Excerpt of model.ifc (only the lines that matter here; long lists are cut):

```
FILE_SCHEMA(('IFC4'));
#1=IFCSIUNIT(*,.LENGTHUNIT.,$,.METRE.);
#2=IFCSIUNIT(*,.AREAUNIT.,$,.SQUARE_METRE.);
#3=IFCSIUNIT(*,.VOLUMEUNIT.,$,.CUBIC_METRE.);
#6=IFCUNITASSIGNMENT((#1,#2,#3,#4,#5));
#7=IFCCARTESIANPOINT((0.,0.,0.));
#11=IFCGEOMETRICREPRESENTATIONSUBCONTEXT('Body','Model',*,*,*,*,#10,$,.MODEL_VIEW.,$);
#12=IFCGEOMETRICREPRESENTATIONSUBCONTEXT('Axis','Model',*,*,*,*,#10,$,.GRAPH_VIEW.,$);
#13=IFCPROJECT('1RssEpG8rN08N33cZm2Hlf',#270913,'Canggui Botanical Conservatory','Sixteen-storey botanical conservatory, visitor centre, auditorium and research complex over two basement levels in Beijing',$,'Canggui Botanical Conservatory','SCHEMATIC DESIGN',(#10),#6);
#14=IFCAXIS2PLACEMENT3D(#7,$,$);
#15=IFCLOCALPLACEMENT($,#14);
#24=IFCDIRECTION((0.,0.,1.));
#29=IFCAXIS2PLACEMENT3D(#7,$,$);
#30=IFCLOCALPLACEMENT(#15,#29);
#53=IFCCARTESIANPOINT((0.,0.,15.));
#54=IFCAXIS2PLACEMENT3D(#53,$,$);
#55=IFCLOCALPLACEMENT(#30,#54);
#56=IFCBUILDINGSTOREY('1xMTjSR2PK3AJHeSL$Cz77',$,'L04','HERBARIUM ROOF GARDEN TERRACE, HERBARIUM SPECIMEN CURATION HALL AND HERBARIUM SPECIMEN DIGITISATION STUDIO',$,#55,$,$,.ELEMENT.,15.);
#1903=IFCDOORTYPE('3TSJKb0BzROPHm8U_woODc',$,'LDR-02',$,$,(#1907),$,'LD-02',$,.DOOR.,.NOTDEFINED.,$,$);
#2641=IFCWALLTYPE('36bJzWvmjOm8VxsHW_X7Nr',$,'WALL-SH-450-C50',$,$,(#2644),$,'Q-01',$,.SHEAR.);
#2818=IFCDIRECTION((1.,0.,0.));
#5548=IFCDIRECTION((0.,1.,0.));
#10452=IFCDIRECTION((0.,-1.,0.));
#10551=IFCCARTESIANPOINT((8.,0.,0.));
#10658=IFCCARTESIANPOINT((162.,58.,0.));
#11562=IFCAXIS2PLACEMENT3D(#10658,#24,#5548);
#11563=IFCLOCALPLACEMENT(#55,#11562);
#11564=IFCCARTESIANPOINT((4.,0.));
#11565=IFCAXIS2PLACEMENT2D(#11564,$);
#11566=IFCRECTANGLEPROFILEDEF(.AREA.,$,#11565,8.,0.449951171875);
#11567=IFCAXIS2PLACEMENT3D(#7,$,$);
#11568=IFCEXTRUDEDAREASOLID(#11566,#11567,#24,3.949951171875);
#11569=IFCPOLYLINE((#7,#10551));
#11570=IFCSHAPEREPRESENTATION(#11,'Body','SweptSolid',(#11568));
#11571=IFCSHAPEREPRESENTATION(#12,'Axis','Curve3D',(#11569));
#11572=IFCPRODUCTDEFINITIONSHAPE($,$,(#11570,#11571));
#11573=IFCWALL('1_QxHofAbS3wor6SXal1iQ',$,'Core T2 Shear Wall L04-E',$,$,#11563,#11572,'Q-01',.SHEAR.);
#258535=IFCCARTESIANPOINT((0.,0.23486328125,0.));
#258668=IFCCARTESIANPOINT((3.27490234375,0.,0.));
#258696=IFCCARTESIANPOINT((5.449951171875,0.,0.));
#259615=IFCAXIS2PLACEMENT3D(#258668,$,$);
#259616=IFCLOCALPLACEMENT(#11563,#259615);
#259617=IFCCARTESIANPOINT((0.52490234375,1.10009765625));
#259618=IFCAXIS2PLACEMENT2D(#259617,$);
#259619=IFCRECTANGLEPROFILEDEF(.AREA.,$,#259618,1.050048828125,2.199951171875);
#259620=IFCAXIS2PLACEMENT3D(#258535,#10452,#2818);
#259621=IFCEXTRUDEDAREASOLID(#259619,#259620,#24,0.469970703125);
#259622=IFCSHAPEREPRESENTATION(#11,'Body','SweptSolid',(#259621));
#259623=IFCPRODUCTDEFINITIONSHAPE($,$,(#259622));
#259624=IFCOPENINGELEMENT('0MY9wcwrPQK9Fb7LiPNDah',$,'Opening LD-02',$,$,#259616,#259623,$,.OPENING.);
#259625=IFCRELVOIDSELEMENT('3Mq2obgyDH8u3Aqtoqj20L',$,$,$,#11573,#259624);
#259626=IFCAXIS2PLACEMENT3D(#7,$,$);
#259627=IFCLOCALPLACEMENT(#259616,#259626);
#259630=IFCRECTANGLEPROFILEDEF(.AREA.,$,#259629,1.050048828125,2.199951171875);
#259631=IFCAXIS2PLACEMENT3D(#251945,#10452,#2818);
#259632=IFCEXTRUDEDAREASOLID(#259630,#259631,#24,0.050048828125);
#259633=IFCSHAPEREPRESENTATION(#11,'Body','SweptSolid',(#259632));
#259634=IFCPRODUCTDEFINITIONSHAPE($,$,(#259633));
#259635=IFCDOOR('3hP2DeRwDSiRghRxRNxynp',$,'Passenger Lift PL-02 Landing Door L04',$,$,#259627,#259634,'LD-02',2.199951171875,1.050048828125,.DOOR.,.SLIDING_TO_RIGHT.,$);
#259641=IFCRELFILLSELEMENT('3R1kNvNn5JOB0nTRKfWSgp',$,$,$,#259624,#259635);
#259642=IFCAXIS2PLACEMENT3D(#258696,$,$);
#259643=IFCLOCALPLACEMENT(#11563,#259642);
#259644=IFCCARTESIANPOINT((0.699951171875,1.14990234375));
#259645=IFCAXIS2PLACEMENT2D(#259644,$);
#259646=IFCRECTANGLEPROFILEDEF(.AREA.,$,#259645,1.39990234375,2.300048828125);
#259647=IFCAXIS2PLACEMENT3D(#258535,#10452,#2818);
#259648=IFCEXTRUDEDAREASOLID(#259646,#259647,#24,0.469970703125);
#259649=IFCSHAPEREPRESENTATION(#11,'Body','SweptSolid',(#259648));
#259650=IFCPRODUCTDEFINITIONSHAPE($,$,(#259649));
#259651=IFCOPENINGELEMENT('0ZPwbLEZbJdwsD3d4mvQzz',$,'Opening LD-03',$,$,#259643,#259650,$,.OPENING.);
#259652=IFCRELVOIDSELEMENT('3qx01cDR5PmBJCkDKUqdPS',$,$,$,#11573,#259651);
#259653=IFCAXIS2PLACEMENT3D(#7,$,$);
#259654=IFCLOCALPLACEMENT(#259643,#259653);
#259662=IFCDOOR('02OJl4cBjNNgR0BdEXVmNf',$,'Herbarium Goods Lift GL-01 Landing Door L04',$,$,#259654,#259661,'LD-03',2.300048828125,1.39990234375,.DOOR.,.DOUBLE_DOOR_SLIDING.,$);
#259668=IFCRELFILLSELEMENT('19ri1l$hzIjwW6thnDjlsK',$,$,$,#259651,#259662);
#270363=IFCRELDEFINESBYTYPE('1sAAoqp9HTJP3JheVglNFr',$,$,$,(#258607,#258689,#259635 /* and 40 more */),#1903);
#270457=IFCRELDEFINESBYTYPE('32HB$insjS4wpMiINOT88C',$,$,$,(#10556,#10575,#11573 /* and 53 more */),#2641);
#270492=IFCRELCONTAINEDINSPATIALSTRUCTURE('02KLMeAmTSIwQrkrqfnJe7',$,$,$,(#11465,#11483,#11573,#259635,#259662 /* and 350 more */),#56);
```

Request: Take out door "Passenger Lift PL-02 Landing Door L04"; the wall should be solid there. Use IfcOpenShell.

```python
import ifcopenshell
import ifcopenshell.api.feature
import ifcopenshell.api.root
import ifcopenshell.geom
import ifcopenshell.util.shape

model = ifcopenshell.open("model.ifc")
settings = ifcopenshell.geom.settings()


def volume(element):
    """Net volume in cubic metres, openings subtracted."""
    shape = ifcopenshell.geom.create_shape(settings, element)
    return ifcopenshell.util.shape.get_volume(shape.geometry)


door = model.by_guid("3hP2DeRwDSiRghRxRNxynp")
opening = door.FillsVoids[0].RelatingOpeningElement
wall = opening.VoidsElements[0].RelatingBuildingElement
before = volume(wall)

ifcopenshell.api.root.remove_product(model, product=door)
ifcopenshell.api.feature.remove_feature(model, feature=opening)

after = volume(wall)

print(f"wall volume {before:.3f} -> {after:.3f} m3")

model.write("model_rev.ifc")
```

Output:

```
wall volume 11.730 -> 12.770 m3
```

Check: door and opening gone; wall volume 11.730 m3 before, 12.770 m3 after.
